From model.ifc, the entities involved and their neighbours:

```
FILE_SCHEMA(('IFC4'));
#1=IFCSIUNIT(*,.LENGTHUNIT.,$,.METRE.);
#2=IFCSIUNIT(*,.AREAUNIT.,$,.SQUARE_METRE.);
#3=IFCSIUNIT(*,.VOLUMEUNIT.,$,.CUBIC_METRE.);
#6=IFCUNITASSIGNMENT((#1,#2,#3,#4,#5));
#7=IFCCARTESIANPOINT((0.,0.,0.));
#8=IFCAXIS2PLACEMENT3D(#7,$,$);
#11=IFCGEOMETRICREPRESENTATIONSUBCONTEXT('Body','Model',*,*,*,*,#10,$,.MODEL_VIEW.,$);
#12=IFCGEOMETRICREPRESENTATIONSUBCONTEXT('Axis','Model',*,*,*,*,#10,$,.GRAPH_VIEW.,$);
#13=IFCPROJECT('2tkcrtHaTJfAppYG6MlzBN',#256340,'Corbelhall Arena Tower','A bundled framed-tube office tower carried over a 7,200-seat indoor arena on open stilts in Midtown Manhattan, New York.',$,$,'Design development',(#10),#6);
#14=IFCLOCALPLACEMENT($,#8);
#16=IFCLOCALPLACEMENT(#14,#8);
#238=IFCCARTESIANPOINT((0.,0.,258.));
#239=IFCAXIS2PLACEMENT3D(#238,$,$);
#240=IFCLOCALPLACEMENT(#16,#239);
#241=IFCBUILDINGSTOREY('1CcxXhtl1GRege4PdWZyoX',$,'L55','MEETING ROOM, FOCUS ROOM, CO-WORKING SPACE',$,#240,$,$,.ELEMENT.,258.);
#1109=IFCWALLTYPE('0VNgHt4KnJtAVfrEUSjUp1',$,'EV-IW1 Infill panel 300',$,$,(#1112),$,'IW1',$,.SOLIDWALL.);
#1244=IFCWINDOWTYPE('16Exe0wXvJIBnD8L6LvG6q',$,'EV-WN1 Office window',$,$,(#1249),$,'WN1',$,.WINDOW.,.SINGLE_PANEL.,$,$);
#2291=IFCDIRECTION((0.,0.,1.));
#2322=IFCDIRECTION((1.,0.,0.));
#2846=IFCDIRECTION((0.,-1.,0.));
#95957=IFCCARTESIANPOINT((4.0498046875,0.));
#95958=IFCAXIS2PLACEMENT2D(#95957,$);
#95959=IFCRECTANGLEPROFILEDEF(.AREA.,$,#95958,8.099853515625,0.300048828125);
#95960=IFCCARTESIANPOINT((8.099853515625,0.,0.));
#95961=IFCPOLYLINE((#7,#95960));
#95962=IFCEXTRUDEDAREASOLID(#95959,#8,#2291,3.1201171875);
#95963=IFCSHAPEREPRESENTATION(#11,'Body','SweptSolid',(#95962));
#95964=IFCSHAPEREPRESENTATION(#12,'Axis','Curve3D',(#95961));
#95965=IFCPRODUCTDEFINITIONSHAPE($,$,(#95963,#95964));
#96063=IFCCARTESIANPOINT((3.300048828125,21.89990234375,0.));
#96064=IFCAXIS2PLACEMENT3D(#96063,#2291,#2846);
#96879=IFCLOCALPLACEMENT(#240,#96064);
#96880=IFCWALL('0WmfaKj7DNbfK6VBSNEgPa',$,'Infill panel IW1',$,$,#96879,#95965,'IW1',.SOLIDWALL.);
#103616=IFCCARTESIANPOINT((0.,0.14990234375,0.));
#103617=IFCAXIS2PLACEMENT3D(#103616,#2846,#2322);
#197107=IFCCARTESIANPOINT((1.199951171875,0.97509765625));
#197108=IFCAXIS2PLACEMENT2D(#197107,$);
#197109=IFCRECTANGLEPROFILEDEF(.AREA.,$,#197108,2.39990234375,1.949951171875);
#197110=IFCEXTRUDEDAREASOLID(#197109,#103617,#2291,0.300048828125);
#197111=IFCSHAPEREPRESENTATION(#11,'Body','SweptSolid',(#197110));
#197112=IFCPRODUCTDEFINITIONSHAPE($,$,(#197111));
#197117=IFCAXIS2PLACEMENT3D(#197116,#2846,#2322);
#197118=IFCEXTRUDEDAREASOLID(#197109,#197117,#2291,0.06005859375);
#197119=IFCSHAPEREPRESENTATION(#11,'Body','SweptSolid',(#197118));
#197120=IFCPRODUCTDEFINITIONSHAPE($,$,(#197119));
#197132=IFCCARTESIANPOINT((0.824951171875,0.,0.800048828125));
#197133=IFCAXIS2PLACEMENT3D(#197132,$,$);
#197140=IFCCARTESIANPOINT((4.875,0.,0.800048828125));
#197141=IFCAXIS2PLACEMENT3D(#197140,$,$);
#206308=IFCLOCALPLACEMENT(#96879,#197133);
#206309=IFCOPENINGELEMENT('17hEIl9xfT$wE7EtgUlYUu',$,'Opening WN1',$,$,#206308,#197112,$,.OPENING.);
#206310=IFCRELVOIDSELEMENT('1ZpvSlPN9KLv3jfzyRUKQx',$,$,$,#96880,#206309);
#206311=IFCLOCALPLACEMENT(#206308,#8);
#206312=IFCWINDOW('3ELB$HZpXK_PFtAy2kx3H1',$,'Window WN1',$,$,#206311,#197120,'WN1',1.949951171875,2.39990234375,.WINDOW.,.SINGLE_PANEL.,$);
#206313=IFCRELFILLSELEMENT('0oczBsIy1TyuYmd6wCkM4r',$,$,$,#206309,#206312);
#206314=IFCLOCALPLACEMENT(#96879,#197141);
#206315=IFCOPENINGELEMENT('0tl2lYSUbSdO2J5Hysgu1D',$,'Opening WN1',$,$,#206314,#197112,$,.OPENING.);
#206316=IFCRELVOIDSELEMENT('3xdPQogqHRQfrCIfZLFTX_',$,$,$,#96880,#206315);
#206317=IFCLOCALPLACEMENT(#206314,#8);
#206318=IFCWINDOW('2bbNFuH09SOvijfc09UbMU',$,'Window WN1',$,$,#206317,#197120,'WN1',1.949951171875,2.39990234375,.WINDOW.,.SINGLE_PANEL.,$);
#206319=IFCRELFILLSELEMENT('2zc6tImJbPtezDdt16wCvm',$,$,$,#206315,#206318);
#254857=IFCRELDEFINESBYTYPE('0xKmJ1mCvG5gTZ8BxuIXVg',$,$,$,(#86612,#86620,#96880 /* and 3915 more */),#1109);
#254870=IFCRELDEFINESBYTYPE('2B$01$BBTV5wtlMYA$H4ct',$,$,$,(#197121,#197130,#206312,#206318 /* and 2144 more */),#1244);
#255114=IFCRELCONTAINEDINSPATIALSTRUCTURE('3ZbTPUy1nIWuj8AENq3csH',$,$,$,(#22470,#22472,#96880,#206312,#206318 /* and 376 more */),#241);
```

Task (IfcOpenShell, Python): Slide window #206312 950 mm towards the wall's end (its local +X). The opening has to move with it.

```python
import ifcopenshell
import ifcopenshell.api.geometry
import ifcopenshell.util.placement
import ifcopenshell.util.unit

model = ifcopenshell.open("model.ifc")
unit_scale = ifcopenshell.util.unit.calculate_unit_scale(model)

window = model.by_guid("3ELB$HZpXK_PFtAy2kx3H1")
opening = window.FillsVoids[0].RelatingOpeningElement
wall = opening.VoidsElements[0].RelatingBuildingElement

wall_matrix = ifcopenshell.util.placement.get_local_placement(wall.ObjectPlacement)
shift = wall_matrix[:3, 0] * 0.95 / unit_scale
before = ifcopenshell.util.placement.get_local_placement(window.ObjectPlacement)[:3, 3].copy()

# The window is placed relative to its opening, so it follows when the opening moves.
matrix = ifcopenshell.util.placement.get_local_placement(opening.ObjectPlacement)
matrix[:3, 3] += shift
ifcopenshell.api.geometry.edit_object_placement(
    model, product=opening, matrix=matrix, is_si=False, should_transform_children=True
)

after = ifcopenshell.util.placement.get_local_placement(window.ObjectPlacement)[:3, 3]
print("window moved by", (after - before).round(3) + 0.0)

model.write("model_updated.ifc")
```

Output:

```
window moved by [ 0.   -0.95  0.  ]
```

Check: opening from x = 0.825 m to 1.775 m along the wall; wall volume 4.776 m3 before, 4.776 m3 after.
